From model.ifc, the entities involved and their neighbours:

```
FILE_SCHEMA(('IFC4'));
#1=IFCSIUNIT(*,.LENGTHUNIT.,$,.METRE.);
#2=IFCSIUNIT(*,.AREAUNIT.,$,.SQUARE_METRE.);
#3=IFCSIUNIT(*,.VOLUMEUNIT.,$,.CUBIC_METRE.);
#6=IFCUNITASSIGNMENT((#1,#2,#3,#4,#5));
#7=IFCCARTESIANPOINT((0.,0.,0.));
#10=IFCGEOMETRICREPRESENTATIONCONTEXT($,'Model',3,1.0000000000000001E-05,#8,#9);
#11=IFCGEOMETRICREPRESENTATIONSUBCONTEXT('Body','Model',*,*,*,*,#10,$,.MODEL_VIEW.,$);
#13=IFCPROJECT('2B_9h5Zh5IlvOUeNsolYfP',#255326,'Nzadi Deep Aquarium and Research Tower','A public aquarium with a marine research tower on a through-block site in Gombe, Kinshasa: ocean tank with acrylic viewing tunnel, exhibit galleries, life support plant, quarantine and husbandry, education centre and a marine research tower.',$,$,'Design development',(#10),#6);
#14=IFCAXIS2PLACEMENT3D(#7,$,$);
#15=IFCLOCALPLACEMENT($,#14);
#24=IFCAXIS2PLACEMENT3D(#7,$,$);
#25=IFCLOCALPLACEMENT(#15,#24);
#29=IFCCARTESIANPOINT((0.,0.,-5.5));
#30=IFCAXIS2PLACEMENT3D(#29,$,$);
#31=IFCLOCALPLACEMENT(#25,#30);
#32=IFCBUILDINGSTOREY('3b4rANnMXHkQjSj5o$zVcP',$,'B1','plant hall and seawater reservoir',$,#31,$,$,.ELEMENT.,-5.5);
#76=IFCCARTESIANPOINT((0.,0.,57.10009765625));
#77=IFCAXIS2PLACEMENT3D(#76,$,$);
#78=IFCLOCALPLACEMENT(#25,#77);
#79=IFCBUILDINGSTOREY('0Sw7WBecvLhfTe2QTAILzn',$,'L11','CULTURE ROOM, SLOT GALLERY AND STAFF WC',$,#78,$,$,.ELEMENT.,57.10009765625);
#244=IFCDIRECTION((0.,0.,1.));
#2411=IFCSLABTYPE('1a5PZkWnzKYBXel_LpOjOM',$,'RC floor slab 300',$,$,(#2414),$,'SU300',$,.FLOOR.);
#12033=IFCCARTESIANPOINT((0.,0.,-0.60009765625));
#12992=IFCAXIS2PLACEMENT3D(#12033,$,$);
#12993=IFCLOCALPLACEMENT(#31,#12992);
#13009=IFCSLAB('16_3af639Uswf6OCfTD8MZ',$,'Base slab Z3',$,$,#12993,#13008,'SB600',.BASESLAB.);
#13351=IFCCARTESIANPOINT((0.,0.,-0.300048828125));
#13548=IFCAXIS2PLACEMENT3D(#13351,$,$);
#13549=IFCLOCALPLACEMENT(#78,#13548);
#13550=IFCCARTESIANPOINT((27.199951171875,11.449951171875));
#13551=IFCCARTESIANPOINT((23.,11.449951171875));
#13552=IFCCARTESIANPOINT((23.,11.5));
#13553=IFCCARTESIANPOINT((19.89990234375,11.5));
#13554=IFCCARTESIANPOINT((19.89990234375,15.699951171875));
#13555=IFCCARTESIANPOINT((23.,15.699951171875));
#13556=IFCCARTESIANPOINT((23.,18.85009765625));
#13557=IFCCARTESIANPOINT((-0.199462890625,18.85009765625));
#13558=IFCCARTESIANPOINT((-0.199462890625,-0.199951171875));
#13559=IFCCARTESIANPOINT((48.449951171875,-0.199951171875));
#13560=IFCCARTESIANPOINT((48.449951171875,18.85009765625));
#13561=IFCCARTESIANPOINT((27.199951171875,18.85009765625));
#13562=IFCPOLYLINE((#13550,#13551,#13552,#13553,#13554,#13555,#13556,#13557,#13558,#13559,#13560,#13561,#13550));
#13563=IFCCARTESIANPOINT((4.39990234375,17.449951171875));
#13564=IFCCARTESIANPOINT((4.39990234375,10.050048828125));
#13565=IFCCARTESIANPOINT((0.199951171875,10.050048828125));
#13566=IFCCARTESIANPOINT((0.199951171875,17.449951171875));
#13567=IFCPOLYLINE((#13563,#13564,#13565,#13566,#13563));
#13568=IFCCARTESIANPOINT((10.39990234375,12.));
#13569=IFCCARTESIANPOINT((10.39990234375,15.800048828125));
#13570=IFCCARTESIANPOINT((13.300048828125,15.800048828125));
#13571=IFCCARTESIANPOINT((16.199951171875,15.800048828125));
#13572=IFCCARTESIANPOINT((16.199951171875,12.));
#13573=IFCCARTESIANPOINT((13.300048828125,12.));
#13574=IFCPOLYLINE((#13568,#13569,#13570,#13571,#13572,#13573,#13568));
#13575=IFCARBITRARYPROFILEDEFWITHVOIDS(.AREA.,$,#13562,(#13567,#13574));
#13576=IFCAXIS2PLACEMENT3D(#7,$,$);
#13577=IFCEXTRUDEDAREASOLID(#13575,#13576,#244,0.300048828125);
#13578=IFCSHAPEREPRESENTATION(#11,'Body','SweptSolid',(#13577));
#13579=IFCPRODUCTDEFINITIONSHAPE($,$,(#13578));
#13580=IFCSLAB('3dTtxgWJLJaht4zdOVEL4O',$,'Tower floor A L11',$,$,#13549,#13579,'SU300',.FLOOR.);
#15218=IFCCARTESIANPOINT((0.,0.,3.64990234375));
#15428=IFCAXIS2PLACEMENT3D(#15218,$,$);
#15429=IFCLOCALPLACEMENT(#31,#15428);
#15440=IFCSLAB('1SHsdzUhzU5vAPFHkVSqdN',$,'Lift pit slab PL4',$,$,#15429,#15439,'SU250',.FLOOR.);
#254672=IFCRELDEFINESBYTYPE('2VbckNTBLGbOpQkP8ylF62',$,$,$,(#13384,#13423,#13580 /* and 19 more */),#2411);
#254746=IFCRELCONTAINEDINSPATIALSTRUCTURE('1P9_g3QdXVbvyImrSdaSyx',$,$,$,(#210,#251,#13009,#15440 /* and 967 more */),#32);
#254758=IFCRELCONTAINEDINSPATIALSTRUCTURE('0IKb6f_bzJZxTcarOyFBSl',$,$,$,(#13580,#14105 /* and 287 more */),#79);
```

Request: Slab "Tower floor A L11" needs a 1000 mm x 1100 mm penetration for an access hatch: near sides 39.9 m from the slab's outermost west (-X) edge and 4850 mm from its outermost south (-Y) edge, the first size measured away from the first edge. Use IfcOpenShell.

```python
import numpy as np
import ifcopenshell
import ifcopenshell.api.feature
import ifcopenshell.api.geometry
import ifcopenshell.api.root
import ifcopenshell.geom
import ifcopenshell.util.placement
import ifcopenshell.util.representation
import ifcopenshell.util.shape
import ifcopenshell.util.unit

model = ifcopenshell.open("model.ifc")
unit_scale = ifcopenshell.util.unit.calculate_unit_scale(model)
settings = ifcopenshell.geom.settings()


def volume(element):
    """Net volume in cubic metres, openings subtracted."""
    shape = ifcopenshell.geom.create_shape(settings, element)
    return ifcopenshell.util.shape.get_volume(shape.geometry)


slab = model.by_guid("3dTtxgWJLJaht4zdOVEL4O")
before = volume(slab)

# Extent in the slab's own axes, in metres. The edges named are its -X and -Y sides.
slab_shape = ifcopenshell.geom.create_shape(settings, slab)
vertices = ifcopenshell.util.shape.get_vertices(slab_shape.geometry)
x_min, y_min, bottom = vertices.min(axis=0)
top = vertices[:, 2].max()

opening = ifcopenshell.api.root.create_entity(model, ifc_class="IfcOpeningElement", name="Access hatch opening", predefined_type="OPENING")
context = ifcopenshell.util.representation.get_context(model, "Model", "Body", "MODEL_VIEW")
width, depth = 1, 1.1
outline = [(0.0, 0.0), (width, 0.0), (width, depth), (0.0, depth), (0.0, 0.0)]
# Overshoot both faces by 50 mm so the cut is clean.
shape = ifcopenshell.api.geometry.add_slab_representation(
    model, context=context, depth=top - bottom + 0.1, polyline=outline
)
ifcopenshell.api.geometry.assign_representation(model, product=opening, representation=shape)

matrix = ifcopenshell.util.placement.get_local_placement(slab.ObjectPlacement)
matrix[:, 3] = matrix @ np.append(np.array([x_min + 39.9, y_min + 4.85, bottom - 0.05]) / unit_scale, 1.0)
ifcopenshell.api.geometry.edit_object_placement(model, product=opening, matrix=matrix, is_si=False)
ifcopenshell.api.feature.add_feature(model, feature=opening, element=slab)

after = volume(slab)

print(f"slab volume {before:.3f} -> {after:.3f} m3")

model.write("model_rev.ifc")
```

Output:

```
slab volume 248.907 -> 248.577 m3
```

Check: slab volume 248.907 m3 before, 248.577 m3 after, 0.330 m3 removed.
